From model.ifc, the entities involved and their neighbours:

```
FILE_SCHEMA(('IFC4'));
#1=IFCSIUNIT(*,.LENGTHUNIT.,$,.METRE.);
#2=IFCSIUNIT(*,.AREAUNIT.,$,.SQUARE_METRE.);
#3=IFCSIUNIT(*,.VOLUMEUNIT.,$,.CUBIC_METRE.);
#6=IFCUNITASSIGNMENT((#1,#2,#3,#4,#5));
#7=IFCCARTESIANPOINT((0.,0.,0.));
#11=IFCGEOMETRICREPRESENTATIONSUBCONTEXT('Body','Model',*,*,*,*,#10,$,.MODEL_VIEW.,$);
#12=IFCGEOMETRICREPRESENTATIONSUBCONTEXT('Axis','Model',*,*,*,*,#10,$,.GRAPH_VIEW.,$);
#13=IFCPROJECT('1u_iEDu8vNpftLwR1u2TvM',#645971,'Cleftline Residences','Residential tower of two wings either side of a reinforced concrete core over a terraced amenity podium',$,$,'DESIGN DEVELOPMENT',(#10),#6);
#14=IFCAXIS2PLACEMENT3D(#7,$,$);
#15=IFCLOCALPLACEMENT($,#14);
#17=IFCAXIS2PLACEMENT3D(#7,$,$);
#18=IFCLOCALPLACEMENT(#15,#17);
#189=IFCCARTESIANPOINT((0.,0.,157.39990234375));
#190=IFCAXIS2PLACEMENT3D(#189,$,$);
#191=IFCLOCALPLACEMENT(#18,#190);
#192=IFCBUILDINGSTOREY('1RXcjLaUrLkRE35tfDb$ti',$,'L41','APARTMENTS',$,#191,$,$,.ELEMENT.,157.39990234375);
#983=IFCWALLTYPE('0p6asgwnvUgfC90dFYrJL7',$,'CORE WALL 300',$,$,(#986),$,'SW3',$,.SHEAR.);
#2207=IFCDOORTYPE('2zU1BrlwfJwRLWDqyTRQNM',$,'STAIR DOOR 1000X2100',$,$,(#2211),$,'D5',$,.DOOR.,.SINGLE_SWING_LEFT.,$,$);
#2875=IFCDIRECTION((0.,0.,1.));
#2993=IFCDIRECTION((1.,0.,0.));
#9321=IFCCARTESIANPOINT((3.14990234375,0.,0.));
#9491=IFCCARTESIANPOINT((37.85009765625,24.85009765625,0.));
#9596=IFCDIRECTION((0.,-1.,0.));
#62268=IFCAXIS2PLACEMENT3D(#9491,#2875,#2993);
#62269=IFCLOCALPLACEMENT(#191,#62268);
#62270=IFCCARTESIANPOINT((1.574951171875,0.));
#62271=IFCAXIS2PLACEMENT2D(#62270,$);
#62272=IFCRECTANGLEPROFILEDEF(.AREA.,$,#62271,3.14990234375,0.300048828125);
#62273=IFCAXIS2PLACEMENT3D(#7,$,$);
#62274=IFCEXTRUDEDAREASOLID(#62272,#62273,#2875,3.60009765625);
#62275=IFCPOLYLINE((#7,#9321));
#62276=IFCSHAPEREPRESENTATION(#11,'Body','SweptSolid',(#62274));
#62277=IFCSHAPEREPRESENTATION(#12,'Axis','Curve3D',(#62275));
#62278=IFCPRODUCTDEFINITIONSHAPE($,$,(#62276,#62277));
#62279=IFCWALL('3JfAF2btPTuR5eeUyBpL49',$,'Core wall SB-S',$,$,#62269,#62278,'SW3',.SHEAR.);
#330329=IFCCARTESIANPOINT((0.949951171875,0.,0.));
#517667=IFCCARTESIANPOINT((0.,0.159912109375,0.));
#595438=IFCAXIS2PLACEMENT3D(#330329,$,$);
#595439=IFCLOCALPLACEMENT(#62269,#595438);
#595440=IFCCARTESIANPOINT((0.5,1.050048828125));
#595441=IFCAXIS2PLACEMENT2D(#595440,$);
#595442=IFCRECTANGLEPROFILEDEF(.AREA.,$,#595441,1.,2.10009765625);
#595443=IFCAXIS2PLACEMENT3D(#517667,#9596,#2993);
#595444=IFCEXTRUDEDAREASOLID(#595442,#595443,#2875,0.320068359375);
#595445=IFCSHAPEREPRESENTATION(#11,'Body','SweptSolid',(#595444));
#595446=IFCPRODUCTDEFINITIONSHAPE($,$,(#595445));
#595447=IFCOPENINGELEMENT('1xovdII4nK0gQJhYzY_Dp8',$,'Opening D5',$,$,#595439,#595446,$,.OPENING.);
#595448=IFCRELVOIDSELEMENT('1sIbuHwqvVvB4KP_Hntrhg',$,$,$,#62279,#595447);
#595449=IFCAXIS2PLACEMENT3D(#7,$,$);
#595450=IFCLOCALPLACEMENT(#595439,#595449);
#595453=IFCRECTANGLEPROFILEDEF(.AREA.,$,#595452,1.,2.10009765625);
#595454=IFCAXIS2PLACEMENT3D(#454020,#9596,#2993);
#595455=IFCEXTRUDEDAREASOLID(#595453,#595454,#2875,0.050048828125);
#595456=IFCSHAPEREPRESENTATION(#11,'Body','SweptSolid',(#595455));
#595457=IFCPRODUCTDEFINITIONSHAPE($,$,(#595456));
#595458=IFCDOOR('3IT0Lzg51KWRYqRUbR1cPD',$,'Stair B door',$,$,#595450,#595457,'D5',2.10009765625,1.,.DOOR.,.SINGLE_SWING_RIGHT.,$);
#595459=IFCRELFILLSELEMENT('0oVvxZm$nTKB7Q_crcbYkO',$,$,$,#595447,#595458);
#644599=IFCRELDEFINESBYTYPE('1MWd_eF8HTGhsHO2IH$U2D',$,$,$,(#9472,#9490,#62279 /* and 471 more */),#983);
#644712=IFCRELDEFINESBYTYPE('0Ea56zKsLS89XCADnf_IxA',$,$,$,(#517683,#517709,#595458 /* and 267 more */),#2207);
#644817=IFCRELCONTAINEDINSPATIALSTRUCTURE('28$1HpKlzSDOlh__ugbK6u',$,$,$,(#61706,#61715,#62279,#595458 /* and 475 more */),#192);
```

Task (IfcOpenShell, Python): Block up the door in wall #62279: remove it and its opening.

```python
import ifcopenshell
import ifcopenshell.api.feature
import ifcopenshell.api.root
import ifcopenshell.geom
import ifcopenshell.util.shape

model = ifcopenshell.open("model.ifc")
settings = ifcopenshell.geom.settings()


def volume(element):
    """Net volume in cubic metres, openings subtracted."""
    shape = ifcopenshell.geom.create_shape(settings, element)
    return ifcopenshell.util.shape.get_volume(shape.geometry)


door = model.by_guid("3IT0Lzg51KWRYqRUbR1cPD")
opening = door.FillsVoids[0].RelatingOpeningElement
wall = opening.VoidsElements[0].RelatingBuildingElement
before = volume(wall)

ifcopenshell.api.root.remove_product(model, product=door)
ifcopenshell.api.feature.remove_feature(model, feature=opening)

after = volume(wall)

print(f"wall volume {before:.3f} -> {after:.3f} m3")

model.write("model-out.ifc")
```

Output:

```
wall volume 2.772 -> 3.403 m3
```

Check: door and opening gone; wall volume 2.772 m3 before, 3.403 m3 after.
